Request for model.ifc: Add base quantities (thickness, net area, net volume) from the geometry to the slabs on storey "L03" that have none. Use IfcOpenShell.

First a look at what the model holds.

```python
import ifcopenshell
import ifcopenshell.util.element
import ifcopenshell.util.unit

model = ifcopenshell.open("model.ifc")
print(model.schema)
for unit_type in ("LENGTHUNIT", "AREAUNIT", "VOLUMEUNIT"):
    print(unit_type, ifcopenshell.util.unit.calculate_unit_scale(model, unit_type))
storey = next(s for s in model.by_type("IfcBuildingStorey") if s.Name == "L03")
slabs = [e for e in ifcopenshell.util.element.get_decomposition(storey) if e.is_a("IfcSlab")]
for e in sorted(slabs, key=lambda e: e.id()):
    print(e.id(), e.is_a(), e.Name, list(ifcopenshell.util.element.get_psets(e, qtos_only=True)), sep=" | ")
```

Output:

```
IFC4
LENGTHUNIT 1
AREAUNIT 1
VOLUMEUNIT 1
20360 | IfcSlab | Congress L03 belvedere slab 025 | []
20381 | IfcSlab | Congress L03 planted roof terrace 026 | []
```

```python
import ifcopenshell
import ifcopenshell.api.pset
import ifcopenshell.geom
import ifcopenshell.util.element
import ifcopenshell.util.shape
import ifcopenshell.util.unit

model = ifcopenshell.open("model.ifc")
unit_scale = ifcopenshell.util.unit.calculate_unit_scale(model)
area_scale = ifcopenshell.util.unit.calculate_unit_scale(model, "AREAUNIT")
volume_scale = ifcopenshell.util.unit.calculate_unit_scale(model, "VOLUMEUNIT")
settings = ifcopenshell.geom.settings()

storey = next(s for s in model.by_type("IfcBuildingStorey") if s.Name == "L03")
slabs = [e for e in ifcopenshell.util.element.get_decomposition(storey) if e.is_a("IfcSlab")]

for e in sorted(slabs, key=lambda e: e.id()):
    if ifcopenshell.util.element.get_psets(e, qtos_only=True, should_inherit=False):
        continue
    # Geometry comes back in metres, in the element's own axes.
    shape = ifcopenshell.geom.create_shape(settings, e)
    values = {
        "Width": ifcopenshell.util.shape.get_z(shape.geometry) / unit_scale,
        "NetArea": ifcopenshell.util.shape.get_footprint_area(shape.geometry) / area_scale,
        "NetVolume": ifcopenshell.util.shape.get_volume(shape.geometry) / volume_scale,
    }
    qto = ifcopenshell.api.pset.add_qto(model, product=e, name="Qto_SlabBaseQuantities")
    ifcopenshell.api.pset.edit_qto(model, qto=qto, properties=values)
    print(e.id(), {k: round(v, 3) for k, v in values.items()})

model.write("model-out.ifc")
```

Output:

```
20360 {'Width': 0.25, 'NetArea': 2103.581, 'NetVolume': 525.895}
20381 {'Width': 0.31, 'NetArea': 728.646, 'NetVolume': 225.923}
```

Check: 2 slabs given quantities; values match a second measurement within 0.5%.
